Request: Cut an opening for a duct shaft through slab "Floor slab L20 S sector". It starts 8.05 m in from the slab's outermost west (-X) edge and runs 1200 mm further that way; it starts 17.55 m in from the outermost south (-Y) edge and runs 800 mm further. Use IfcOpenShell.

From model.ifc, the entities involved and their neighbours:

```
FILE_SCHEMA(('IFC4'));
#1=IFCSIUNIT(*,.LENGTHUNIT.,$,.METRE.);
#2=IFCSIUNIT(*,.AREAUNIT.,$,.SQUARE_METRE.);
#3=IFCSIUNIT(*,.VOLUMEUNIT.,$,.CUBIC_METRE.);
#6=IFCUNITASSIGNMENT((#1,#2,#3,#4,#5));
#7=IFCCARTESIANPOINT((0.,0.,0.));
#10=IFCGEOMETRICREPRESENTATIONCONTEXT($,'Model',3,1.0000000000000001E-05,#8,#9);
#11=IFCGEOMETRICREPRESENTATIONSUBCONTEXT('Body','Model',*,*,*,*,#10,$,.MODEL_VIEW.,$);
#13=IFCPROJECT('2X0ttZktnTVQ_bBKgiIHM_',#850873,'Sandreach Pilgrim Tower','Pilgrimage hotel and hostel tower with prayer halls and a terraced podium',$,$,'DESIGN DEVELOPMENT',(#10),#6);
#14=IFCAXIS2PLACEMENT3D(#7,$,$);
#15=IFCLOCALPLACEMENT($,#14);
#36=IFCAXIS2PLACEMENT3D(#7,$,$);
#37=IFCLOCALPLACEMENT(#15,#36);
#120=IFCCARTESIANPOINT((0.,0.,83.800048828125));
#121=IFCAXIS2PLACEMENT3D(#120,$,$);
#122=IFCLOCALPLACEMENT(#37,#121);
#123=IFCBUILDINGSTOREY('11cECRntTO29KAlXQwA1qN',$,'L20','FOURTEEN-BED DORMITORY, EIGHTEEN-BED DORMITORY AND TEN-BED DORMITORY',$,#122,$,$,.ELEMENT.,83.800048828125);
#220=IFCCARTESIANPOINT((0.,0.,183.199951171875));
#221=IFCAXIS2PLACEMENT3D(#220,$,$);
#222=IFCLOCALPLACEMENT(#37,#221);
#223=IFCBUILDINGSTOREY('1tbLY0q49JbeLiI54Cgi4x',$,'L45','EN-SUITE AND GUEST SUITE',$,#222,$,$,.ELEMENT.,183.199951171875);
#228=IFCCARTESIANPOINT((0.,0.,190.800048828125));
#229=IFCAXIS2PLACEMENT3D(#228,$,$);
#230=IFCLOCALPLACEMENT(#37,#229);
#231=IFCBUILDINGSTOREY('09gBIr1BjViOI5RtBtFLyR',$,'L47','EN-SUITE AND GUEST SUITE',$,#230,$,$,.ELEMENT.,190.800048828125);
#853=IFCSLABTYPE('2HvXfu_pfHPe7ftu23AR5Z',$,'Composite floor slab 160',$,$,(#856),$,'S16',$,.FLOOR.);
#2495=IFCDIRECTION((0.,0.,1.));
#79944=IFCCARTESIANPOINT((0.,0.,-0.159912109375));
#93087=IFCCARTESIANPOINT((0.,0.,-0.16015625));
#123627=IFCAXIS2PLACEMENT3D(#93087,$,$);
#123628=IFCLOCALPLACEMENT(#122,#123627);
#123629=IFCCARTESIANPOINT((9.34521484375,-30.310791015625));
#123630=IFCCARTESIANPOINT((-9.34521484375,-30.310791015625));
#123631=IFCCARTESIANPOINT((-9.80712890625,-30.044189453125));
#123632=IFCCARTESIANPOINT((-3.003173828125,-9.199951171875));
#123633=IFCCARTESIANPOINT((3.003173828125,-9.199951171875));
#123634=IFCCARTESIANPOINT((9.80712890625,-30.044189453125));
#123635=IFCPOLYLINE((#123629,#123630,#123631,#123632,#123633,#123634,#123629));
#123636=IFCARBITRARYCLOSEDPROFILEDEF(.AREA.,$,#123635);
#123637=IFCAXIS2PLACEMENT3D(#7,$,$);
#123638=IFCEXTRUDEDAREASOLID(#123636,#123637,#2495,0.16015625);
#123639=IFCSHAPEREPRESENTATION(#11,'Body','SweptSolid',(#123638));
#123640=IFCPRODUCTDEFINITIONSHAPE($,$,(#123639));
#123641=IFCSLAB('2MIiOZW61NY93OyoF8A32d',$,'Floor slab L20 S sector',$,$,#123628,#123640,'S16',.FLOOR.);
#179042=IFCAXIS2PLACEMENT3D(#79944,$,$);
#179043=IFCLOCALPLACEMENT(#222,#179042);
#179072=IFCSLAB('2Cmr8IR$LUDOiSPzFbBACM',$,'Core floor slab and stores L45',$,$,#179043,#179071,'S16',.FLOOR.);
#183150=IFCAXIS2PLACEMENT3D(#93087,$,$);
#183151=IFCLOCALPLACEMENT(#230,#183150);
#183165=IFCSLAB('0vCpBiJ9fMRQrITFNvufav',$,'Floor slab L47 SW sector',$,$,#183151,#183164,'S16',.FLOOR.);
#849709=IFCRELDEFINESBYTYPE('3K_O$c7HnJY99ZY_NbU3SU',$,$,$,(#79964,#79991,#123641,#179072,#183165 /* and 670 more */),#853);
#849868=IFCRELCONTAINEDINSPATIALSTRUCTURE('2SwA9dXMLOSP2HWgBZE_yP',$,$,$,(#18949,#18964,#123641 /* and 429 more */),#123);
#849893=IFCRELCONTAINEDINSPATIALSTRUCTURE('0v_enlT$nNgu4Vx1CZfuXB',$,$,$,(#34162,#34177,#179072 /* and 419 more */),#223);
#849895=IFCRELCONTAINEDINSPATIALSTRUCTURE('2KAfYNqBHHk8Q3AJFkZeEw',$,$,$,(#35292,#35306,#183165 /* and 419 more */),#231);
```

```python
import numpy as np
import ifcopenshell
import ifcopenshell.api.feature
import ifcopenshell.api.geometry
import ifcopenshell.api.root
import ifcopenshell.geom
import ifcopenshell.util.placement
import ifcopenshell.util.representation
import ifcopenshell.util.shape
import ifcopenshell.util.unit

model = ifcopenshell.open("model.ifc")
unit_scale = ifcopenshell.util.unit.calculate_unit_scale(model)
settings = ifcopenshell.geom.settings()


def volume(element):
    """Net volume in cubic metres, openings subtracted."""
    shape = ifcopenshell.geom.create_shape(settings, element)
    return ifcopenshell.util.shape.get_volume(shape.geometry)


slab = model.by_id(123641)
before = volume(slab)

# Extent in the slab's own axes, in metres. The edges named are its -X and -Y sides.
slab_shape = ifcopenshell.geom.create_shape(settings, slab)
vertices = ifcopenshell.util.shape.get_vertices(slab_shape.geometry)
x_min, y_min, bottom = vertices.min(axis=0)
top = vertices[:, 2].max()

opening = ifcopenshell.api.root.create_entity(model, ifc_class="IfcOpeningElement", name="Duct shaft opening", predefined_type="OPENING")
context = ifcopenshell.util.representation.get_context(model, "Model", "Body", "MODEL_VIEW")
width, depth = 1.2, 0.8
outline = [(0.0, 0.0), (width, 0.0), (width, depth), (0.0, depth), (0.0, 0.0)]
# Overshoot both faces by 50 mm so the cut is clean.
shape = ifcopenshell.api.geometry.add_slab_representation(
    model, context=context, depth=top - bottom + 0.1, polyline=outline
)
ifcopenshell.api.geometry.assign_representation(model, product=opening, representation=shape)

matrix = ifcopenshell.util.placement.get_local_placement(slab.ObjectPlacement)
matrix[:, 3] = matrix @ np.append(np.array([x_min + 8.05, y_min + 17.55, bottom - 0.05]) / unit_scale, 1.0)
ifcopenshell.api.geometry.edit_object_placement(model, product=opening, matrix=matrix, is_si=False)
ifcopenshell.api.feature.add_feature(model, feature=opening, element=slab)

after = volume(slab)

print(f"slab volume {before:.3f} -> {after:.3f} m3")

model.write("model_rev.ifc")
```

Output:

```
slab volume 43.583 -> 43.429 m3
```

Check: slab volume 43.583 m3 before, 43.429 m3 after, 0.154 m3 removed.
